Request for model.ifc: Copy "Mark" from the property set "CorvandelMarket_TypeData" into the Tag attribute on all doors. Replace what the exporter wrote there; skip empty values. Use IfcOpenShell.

First a look at what the model holds.

```python
import ifcopenshell
import ifcopenshell.util.element

model = ifcopenshell.open("model.ifc")
print(model.schema)
doors = model.by_type("IfcDoor")
print(len(doors), "doors")
for e in doors[:8]:
    source = ifcopenshell.util.element.get_pset(e, "CorvandelMarket_TypeData", "Mark")
    target = e.Tag
    print(e.id(), repr(source), repr(target), sep=" | ")
```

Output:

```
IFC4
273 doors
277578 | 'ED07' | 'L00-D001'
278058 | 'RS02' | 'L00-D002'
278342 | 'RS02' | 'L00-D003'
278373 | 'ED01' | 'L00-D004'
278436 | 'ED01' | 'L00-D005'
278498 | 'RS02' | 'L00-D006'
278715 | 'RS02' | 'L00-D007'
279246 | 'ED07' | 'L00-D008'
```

```python
import ifcopenshell
import ifcopenshell.util.element

model = ifcopenshell.open("model.ifc")

count = 0
for e in model.by_type("IfcDoor"):
    value = ifcopenshell.util.element.get_pset(e, "CorvandelMarket_TypeData", "Mark")
    current = e.Tag
    if not value or not value.strip() or current == value:
        continue
    e.Tag = value
    count += 1

print(count, "doors updated")

model.write("model-out.ifc")
```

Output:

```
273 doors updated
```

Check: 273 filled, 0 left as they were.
